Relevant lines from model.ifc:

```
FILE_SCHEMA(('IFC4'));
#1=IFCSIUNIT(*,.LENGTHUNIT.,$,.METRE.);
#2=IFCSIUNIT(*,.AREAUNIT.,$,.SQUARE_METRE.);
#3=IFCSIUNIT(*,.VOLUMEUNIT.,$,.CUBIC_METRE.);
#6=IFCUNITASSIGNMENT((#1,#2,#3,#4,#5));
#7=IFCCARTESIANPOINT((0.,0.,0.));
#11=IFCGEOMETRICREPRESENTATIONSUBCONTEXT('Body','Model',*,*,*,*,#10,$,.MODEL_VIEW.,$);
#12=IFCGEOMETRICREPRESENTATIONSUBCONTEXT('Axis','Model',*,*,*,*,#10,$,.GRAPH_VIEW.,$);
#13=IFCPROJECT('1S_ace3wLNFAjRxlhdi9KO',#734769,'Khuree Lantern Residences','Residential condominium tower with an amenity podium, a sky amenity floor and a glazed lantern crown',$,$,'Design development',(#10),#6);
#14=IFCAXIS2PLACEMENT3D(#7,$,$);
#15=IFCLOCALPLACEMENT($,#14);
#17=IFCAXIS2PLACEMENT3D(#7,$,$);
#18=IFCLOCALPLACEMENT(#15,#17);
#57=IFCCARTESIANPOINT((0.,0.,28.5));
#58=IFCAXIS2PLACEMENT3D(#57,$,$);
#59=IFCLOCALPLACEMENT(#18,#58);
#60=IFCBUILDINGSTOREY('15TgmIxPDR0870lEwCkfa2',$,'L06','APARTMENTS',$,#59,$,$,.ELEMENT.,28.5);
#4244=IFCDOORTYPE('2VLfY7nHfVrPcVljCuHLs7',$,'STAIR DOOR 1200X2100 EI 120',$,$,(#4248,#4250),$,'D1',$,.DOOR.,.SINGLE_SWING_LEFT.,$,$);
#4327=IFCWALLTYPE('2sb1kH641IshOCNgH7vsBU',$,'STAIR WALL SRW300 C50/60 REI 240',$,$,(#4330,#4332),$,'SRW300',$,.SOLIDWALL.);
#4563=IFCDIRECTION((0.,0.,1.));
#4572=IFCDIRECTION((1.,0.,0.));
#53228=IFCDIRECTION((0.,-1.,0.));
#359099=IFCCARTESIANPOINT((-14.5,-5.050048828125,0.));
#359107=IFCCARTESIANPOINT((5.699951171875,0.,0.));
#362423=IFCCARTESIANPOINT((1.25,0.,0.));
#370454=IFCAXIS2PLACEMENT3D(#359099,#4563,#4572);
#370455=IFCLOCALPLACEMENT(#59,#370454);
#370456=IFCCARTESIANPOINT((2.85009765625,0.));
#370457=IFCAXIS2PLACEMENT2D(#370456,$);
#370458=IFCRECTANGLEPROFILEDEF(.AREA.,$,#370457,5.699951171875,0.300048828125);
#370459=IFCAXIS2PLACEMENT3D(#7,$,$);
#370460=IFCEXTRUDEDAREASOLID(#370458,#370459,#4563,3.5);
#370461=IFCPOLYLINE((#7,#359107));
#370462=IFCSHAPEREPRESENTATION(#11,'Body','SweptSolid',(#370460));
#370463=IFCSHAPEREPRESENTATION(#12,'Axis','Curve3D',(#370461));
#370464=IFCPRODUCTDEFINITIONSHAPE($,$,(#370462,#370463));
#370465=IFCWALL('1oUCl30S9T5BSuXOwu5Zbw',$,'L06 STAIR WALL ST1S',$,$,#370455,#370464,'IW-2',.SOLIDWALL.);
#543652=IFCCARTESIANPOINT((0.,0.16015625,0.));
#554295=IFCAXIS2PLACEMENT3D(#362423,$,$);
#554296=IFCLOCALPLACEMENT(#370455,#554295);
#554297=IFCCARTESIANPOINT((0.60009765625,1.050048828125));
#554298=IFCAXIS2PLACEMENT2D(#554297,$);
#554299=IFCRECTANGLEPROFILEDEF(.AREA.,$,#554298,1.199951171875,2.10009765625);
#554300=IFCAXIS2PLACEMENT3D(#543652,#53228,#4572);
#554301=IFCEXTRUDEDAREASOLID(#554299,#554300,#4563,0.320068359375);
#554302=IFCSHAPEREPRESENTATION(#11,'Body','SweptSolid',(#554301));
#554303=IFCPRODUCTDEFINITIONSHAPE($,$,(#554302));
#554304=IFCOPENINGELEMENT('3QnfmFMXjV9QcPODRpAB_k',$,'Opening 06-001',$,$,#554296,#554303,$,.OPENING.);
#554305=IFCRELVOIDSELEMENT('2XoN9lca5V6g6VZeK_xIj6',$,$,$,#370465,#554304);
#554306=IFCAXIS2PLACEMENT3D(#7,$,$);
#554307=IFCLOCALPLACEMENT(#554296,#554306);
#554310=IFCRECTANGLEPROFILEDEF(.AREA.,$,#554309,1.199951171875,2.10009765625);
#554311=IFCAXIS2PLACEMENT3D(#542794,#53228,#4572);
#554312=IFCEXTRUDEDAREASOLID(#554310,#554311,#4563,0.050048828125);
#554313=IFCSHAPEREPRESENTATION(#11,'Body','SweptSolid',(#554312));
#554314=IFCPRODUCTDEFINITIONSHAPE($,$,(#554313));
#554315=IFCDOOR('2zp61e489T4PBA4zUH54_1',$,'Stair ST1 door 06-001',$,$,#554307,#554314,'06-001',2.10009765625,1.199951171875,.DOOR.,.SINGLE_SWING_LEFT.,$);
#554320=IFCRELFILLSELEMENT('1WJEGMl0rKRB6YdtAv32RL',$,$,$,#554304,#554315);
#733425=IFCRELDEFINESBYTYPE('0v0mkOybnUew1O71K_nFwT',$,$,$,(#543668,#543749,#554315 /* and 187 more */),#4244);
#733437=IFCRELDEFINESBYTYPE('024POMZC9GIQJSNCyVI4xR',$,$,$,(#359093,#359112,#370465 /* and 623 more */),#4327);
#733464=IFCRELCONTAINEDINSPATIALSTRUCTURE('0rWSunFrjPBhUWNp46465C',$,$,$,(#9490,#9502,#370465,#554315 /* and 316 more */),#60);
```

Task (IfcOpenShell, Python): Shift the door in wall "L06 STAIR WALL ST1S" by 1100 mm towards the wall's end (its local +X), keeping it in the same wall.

```python
import ifcopenshell
import ifcopenshell.api.geometry
import ifcopenshell.util.placement
import ifcopenshell.util.unit

model = ifcopenshell.open("model.ifc")
unit_scale = ifcopenshell.util.unit.calculate_unit_scale(model)

door = model.by_guid("2zp61e489T4PBA4zUH54_1")
opening = door.FillsVoids[0].RelatingOpeningElement
wall = opening.VoidsElements[0].RelatingBuildingElement

wall_matrix = ifcopenshell.util.placement.get_local_placement(wall.ObjectPlacement)
shift = wall_matrix[:3, 0] * 1.1 / unit_scale
before = ifcopenshell.util.placement.get_local_placement(door.ObjectPlacement)[:3, 3].copy()

# The door is placed relative to its opening, so it follows when the opening moves.
matrix = ifcopenshell.util.placement.get_local_placement(opening.ObjectPlacement)
matrix[:3, 3] += shift
ifcopenshell.api.geometry.edit_object_placement(
    model, product=opening, matrix=matrix, is_si=False, should_transform_children=True
)

after = ifcopenshell.util.placement.get_local_placement(door.ObjectPlacement)[:3, 3]
print("door moved by", (after - before).round(3) + 0.0)

model.write("model_rev.ifc")
```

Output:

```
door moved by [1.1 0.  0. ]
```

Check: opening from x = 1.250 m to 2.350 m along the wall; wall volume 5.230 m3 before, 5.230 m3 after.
